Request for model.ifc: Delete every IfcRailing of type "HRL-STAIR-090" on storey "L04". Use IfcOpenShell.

First a look at what the model holds.

```python
import ifcopenshell
import ifcopenshell.util.element

model = ifcopenshell.open("model.ifc")
print(model.schema)
storey = next(s for s in model.by_type("IfcBuildingStorey") if s.Name == "L04")
railings = [e for e in ifcopenshell.util.element.get_decomposition(storey) if e.is_a("IfcRailing")]
seen = {}
for e in railings:
    element_type = ifcopenshell.util.element.get_type(e)
    name = element_type.Name if element_type not in (None, e) else None
    seen[name] = seen.get(name, 0) + 1
for name, count in sorted(seen.items(), key=str):
    print(count, "x", name)
```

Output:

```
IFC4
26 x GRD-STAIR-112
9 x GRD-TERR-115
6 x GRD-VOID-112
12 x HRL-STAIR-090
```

```python
import ifcopenshell
import ifcopenshell.api.root
import ifcopenshell.util.element

model = ifcopenshell.open("model.ifc")

storey = next(s for s in model.by_type("IfcBuildingStorey") if s.Name == "L04")
railings = [e for e in ifcopenshell.util.element.get_decomposition(storey) if e.is_a("IfcRailing")]
targets = [e for e in railings if (t := ifcopenshell.util.element.get_type(e)) not in (None, e) and t.Name == "HRL-STAIR-090"]

for e in targets:
    ifcopenshell.api.root.remove_product(model, product=e)
print(len(targets), "removed")

model.write("model_rev.ifc")
```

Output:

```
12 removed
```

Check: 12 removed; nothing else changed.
